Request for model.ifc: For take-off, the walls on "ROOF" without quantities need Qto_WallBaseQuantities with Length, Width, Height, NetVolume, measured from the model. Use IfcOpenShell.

First a look at what the model holds.

```python
import ifcopenshell
import ifcopenshell.util.element
import ifcopenshell.util.unit

model = ifcopenshell.open("model.ifc")
print(model.schema)
for unit_type in ("LENGTHUNIT", "AREAUNIT", "VOLUMEUNIT"):
    print(unit_type, ifcopenshell.util.unit.calculate_unit_scale(model, unit_type))
storey = next(s for s in model.by_type("IfcBuildingStorey") if s.Name == "ROOF")
walls = [e for e in ifcopenshell.util.element.get_decomposition(storey) if e.is_a("IfcWall")]
for e in sorted(walls, key=lambda e: e.id()):
    print(e.id(), e.is_a(), e.Name, list(ifcopenshell.util.element.get_psets(e, qtos_only=True)), sep=" | ")
```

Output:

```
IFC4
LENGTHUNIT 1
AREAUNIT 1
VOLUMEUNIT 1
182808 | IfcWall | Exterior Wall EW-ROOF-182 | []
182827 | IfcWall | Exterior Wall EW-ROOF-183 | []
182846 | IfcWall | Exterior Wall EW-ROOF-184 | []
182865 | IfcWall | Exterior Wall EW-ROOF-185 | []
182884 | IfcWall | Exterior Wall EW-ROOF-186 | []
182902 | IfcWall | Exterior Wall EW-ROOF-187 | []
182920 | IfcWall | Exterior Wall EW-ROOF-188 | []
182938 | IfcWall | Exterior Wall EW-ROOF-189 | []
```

```python
import ifcopenshell
import ifcopenshell.api.pset
import ifcopenshell.geom
import ifcopenshell.util.element
import ifcopenshell.util.shape
import ifcopenshell.util.unit

model = ifcopenshell.open("model.ifc")
unit_scale = ifcopenshell.util.unit.calculate_unit_scale(model)
volume_scale = ifcopenshell.util.unit.calculate_unit_scale(model, "VOLUMEUNIT")
settings = ifcopenshell.geom.settings()

storey = next(s for s in model.by_type("IfcBuildingStorey") if s.Name == "ROOF")
walls = [e for e in ifcopenshell.util.element.get_decomposition(storey) if e.is_a("IfcWall")]

for e in sorted(walls, key=lambda e: e.id()):
    if ifcopenshell.util.element.get_psets(e, qtos_only=True, should_inherit=False):
        continue
    # Geometry comes back in metres, in the element's own axes.
    shape = ifcopenshell.geom.create_shape(settings, e)
    values = {
        "Length": ifcopenshell.util.shape.get_x(shape.geometry) / unit_scale,
        "Width": ifcopenshell.util.shape.get_y(shape.geometry) / unit_scale,
        "Height": ifcopenshell.util.shape.get_z(shape.geometry) / unit_scale,
        "NetVolume": ifcopenshell.util.shape.get_volume(shape.geometry) / volume_scale,
    }
    qto = ifcopenshell.api.pset.add_qto(model, product=e, name="Qto_WallBaseQuantities")
    ifcopenshell.api.pset.edit_qto(model, qto=qto, properties=values)
    print(e.id(), {k: round(v, 3) for k, v in values.items()})

model.write("model_rev.ifc")
```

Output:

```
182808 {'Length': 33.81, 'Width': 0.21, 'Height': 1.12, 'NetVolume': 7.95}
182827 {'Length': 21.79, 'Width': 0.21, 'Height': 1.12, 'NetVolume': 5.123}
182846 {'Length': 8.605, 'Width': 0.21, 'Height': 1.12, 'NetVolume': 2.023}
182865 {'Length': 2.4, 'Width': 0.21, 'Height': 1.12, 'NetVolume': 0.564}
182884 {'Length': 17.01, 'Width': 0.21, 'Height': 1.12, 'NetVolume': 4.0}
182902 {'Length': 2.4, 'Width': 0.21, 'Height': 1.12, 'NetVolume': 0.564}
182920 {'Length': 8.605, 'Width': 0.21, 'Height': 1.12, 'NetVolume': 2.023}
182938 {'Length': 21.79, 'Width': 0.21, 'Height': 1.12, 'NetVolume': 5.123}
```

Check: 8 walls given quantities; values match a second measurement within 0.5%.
